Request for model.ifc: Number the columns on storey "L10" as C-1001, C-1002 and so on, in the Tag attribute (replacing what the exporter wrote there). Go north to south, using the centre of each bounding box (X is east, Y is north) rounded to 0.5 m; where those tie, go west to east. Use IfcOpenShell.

First a look at what the model holds.

```python
import ifcopenshell
import ifcopenshell.util.element
import ifcopenshell.util.placement

model = ifcopenshell.open("model.ifc")
print(model.schema)
storey = next(s for s in model.by_type("IfcBuildingStorey") if s.Name == "L10")
columns = [e for e in ifcopenshell.util.element.get_decomposition(storey) if e.is_a("IfcColumn")]
for e in sorted(columns, key=lambda e: e.id()):
    origin = ifcopenshell.util.placement.get_local_placement(e.ObjectPlacement)[:3, 3]
    print(e.id(), e.Tag, e.Name, origin.round(2) + 0.0, sep=" | ")
```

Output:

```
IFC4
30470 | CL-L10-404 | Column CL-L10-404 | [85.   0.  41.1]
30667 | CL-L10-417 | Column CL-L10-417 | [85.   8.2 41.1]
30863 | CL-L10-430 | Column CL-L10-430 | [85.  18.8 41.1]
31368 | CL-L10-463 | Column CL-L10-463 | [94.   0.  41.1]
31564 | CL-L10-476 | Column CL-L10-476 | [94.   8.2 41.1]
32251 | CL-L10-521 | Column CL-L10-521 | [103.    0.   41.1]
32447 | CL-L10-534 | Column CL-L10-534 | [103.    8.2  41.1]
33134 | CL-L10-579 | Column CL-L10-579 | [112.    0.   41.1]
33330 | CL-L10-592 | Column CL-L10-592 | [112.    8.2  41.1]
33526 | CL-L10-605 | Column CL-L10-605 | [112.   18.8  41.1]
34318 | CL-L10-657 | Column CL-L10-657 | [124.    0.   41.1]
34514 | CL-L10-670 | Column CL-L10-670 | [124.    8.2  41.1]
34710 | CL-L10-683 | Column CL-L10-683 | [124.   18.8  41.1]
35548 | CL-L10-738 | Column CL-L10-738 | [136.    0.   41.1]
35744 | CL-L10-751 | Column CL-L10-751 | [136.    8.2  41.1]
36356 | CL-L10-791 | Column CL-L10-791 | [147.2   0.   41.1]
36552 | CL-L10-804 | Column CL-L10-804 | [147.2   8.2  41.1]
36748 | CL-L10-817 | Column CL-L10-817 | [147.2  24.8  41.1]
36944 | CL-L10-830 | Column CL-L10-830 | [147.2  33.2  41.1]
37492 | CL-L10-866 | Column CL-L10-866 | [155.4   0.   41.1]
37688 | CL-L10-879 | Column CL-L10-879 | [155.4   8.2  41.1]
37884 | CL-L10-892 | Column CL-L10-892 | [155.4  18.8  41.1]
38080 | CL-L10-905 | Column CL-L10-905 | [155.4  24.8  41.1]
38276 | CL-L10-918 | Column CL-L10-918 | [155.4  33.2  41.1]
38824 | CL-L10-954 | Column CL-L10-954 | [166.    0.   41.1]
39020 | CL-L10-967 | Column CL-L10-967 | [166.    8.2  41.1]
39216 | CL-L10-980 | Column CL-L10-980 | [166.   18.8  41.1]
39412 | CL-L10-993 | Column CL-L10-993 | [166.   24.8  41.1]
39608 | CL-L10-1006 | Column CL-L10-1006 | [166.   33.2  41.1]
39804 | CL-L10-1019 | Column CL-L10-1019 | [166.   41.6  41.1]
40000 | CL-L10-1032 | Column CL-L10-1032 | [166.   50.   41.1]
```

```python
import ifcopenshell
import ifcopenshell.geom
import ifcopenshell.util.element
import ifcopenshell.util.shape

model = ifcopenshell.open("model.ifc")
settings = ifcopenshell.geom.settings()
settings.set("use-world-coords", True)


def centre(element):
    shape = ifcopenshell.geom.create_shape(settings, element)
    return ifcopenshell.util.shape.get_bbox_centroid(shape.geometry)


storey = next(s for s in model.by_type("IfcBuildingStorey") if s.Name == "L10")
columns = [e for e in ifcopenshell.util.element.get_decomposition(storey) if e.is_a("IfcColumn")]

# Insertion points can sit at a corner or the storey origin, so sort by the geometry (in metres).
centres = {e: centre(e) for e in columns}
columns.sort(key=lambda e: (-round(centres[e][1] / 0.5), centres[e][0]))

for i, e in enumerate(columns, start=1):
    number = f"C-10{i:02d}"
    e.Tag = number
    print(e.id(), number)

model.write("model_v2.ifc")
```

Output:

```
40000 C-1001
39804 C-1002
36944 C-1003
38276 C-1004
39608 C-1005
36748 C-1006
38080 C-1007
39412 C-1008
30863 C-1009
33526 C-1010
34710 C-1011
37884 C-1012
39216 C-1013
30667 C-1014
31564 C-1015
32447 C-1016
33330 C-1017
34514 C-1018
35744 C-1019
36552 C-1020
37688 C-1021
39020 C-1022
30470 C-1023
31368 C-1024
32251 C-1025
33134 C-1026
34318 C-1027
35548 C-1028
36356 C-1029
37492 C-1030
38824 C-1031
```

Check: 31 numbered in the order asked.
